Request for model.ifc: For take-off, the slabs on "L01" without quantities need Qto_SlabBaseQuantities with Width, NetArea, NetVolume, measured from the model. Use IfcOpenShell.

First a look at what the model holds.

```python
import ifcopenshell
import ifcopenshell.util.element
import ifcopenshell.util.unit

model = ifcopenshell.open("model.ifc")
print(model.schema)
for unit_type in ("LENGTHUNIT", "AREAUNIT", "VOLUMEUNIT"):
    print(unit_type, ifcopenshell.util.unit.calculate_unit_scale(model, unit_type))
storey = next(s for s in model.by_type("IfcBuildingStorey") if s.Name == "L01")
slabs = [e for e in ifcopenshell.util.element.get_decomposition(storey) if e.is_a("IfcSlab")]
for e in sorted(slabs, key=lambda e: e.id()):
    print(e.id(), e.is_a(), e.Name, list(ifcopenshell.util.element.get_psets(e, qtos_only=True)), sep=" | ")
```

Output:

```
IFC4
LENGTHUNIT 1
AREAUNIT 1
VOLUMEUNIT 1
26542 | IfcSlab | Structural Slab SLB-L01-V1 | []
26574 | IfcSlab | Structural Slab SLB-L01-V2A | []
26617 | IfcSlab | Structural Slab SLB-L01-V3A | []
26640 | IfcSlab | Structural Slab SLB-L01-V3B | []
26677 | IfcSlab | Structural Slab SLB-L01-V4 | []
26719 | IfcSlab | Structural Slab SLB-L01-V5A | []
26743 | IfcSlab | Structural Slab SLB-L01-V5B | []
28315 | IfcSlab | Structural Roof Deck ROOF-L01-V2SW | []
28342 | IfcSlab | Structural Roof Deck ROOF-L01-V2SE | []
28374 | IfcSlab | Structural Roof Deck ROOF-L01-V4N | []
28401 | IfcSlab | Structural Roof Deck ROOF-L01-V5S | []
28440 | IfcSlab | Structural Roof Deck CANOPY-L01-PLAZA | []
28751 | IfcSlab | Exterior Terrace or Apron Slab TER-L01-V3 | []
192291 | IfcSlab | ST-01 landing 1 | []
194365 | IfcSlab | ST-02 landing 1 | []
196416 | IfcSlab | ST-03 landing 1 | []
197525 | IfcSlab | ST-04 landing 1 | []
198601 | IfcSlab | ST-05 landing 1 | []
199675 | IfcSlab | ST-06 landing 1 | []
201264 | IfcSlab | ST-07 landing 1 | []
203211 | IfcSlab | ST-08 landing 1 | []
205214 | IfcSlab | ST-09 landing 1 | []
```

```python
import ifcopenshell
import ifcopenshell.api.pset
import ifcopenshell.geom
import ifcopenshell.util.element
import ifcopenshell.util.shape
import ifcopenshell.util.unit

model = ifcopenshell.open("model.ifc")
unit_scale = ifcopenshell.util.unit.calculate_unit_scale(model)
area_scale = ifcopenshell.util.unit.calculate_unit_scale(model, "AREAUNIT")
volume_scale = ifcopenshell.util.unit.calculate_unit_scale(model, "VOLUMEUNIT")
settings = ifcopenshell.geom.settings()

storey = next(s for s in model.by_type("IfcBuildingStorey") if s.Name == "L01")
slabs = [e for e in ifcopenshell.util.element.get_decomposition(storey) if e.is_a("IfcSlab")]

for e in sorted(slabs, key=lambda e: e.id()):
    if ifcopenshell.util.element.get_psets(e, qtos_only=True, should_inherit=False):
        continue
    # Geometry comes back in metres, in the element's own axes.
    shape = ifcopenshell.geom.create_shape(settings, e)
    values = {
        "Width": ifcopenshell.util.shape.get_z(shape.geometry) / unit_scale,
        "NetArea": ifcopenshell.util.shape.get_footprint_area(shape.geometry) / area_scale,
        "NetVolume": ifcopenshell.util.shape.get_volume(shape.geometry) / volume_scale,
    }
    qto = ifcopenshell.api.pset.add_qto(model, product=e, name="Qto_SlabBaseQuantities")
    ifcopenshell.api.pset.edit_qto(model, qto=qto, properties=values)
    print(e.id(), {k: round(v, 3) for k, v in values.items()})

model.write("model-out.ifc")
```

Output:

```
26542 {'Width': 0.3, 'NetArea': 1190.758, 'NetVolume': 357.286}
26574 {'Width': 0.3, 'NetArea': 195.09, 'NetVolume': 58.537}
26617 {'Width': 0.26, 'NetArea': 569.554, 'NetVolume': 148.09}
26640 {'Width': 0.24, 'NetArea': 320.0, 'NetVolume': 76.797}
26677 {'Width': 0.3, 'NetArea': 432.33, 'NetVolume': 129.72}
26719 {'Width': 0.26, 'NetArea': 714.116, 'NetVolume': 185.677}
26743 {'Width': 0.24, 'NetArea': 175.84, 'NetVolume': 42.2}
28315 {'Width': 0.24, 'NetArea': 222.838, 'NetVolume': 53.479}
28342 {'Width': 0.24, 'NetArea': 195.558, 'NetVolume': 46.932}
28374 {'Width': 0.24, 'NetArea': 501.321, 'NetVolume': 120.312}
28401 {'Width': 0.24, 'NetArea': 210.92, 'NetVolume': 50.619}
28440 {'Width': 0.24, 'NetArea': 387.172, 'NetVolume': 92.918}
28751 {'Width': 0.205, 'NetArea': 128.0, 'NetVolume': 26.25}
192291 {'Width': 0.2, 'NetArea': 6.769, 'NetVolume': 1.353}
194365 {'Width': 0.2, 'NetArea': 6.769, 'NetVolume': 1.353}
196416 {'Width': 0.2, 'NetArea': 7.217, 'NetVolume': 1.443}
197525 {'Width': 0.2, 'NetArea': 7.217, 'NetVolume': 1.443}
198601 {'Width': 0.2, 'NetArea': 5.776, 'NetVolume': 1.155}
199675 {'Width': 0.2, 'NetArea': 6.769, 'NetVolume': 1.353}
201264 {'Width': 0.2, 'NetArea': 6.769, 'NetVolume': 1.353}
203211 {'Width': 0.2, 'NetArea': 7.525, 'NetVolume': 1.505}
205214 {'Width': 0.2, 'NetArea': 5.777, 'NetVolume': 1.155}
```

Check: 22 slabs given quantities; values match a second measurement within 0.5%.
